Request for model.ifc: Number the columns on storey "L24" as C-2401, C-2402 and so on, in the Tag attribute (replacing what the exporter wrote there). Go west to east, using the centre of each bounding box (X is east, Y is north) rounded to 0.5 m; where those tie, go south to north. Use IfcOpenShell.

First a look at what the model holds.

```python
import ifcopenshell
import ifcopenshell.util.element
import ifcopenshell.util.placement

model = ifcopenshell.open("model.ifc")
print(model.schema)
storey = next(s for s in model.by_type("IfcBuildingStorey") if s.Name == "L24")
columns = [e for e in ifcopenshell.util.element.get_decomposition(storey) if e.is_a("IfcColumn")]
for e in sorted(columns, key=lambda e: e.id()):
    origin = ifcopenshell.util.placement.get_local_placement(e.ObjectPlacement)[:3, 3]
    print(e.id(), e.Tag, e.Name, origin.round(2) + 0.0, sep=" | ")
```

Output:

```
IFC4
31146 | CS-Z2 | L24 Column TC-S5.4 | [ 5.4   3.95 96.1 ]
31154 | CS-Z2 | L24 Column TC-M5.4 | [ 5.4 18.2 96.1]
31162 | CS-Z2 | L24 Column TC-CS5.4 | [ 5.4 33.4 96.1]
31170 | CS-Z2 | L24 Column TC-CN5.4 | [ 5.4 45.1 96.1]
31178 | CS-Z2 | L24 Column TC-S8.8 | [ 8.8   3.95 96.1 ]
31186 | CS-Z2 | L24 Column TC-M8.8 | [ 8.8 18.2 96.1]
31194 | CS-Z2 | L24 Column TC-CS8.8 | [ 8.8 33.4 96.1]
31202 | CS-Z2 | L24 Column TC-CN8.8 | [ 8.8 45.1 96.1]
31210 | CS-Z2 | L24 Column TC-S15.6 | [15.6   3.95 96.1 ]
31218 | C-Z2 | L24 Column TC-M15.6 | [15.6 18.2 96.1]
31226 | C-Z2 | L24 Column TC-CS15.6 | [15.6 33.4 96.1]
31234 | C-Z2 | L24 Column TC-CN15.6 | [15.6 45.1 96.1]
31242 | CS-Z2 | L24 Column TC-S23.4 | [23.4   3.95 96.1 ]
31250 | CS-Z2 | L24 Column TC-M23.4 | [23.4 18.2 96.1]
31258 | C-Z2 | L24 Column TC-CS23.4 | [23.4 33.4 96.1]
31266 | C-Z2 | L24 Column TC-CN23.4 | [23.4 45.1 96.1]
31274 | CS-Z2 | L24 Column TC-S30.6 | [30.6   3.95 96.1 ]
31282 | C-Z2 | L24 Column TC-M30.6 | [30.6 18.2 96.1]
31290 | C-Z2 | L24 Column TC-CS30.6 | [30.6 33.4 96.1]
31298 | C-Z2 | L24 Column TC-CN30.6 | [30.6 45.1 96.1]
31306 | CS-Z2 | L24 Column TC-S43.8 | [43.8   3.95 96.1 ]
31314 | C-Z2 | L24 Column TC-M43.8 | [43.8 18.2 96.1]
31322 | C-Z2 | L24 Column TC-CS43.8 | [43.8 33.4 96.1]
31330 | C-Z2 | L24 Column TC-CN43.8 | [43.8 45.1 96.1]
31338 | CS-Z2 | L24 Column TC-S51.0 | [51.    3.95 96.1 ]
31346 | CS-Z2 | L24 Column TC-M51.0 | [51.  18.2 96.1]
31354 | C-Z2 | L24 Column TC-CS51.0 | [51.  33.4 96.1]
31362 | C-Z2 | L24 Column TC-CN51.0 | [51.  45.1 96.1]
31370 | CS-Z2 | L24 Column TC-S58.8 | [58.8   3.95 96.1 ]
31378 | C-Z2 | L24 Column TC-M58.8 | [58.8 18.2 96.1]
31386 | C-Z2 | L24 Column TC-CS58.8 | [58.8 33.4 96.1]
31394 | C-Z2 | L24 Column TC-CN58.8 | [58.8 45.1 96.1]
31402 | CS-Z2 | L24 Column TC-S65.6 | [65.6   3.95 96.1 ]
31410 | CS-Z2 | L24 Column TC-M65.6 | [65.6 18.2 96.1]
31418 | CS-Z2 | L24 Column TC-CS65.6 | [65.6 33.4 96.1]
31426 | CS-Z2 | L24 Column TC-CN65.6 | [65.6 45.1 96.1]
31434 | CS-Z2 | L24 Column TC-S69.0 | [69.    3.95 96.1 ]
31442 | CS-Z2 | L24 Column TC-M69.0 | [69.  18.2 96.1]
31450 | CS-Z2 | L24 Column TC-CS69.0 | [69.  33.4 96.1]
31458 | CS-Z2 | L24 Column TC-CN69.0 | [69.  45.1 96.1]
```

```python
import ifcopenshell
import ifcopenshell.geom
import ifcopenshell.util.element
import ifcopenshell.util.shape

model = ifcopenshell.open("model.ifc")
settings = ifcopenshell.geom.settings()
settings.set("use-world-coords", True)


def centre(element):
    shape = ifcopenshell.geom.create_shape(settings, element)
    return ifcopenshell.util.shape.get_bbox_centroid(shape.geometry)


storey = next(s for s in model.by_type("IfcBuildingStorey") if s.Name == "L24")
columns = [e for e in ifcopenshell.util.element.get_decomposition(storey) if e.is_a("IfcColumn")]

# Insertion points can sit at a corner or the storey origin, so sort by the geometry (in metres).
centres = {e: centre(e) for e in columns}
columns.sort(key=lambda e: (round(centres[e][0] / 0.5), centres[e][1]))

for i, e in enumerate(columns, start=1):
    number = f"C-24{i:02d}"
    e.Tag = number
    print(e.id(), number)

model.write("model_edited.ifc")
```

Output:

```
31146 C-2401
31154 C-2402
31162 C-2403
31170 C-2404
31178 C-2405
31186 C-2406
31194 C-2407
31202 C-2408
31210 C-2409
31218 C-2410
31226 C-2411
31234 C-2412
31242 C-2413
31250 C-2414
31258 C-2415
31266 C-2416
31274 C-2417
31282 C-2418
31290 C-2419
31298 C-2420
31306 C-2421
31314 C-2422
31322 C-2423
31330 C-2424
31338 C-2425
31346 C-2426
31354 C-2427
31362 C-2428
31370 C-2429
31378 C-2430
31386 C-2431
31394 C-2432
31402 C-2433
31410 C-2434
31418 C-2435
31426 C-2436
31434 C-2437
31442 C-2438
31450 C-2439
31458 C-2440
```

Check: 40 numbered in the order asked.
